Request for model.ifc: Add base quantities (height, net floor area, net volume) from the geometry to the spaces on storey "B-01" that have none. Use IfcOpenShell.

First a look at what the model holds.

```python
import ifcopenshell
import ifcopenshell.util.element
import ifcopenshell.util.unit

model = ifcopenshell.open("model.ifc")
print(model.schema)
for unit_type in ("LENGTHUNIT", "AREAUNIT", "VOLUMEUNIT"):
    print(unit_type, ifcopenshell.util.unit.calculate_unit_scale(model, unit_type))
storey = next(s for s in model.by_type("IfcBuildingStorey") if s.Name == "B-01")
spaces = [e for e in ifcopenshell.util.element.get_decomposition(storey) if e.is_a("IfcSpace")]
for e in sorted(spaces, key=lambda e: e.id()):
    print(e.id(), e.is_a(), e.Name, list(ifcopenshell.util.element.get_psets(e, qtos_only=True)), sep=" | ")
```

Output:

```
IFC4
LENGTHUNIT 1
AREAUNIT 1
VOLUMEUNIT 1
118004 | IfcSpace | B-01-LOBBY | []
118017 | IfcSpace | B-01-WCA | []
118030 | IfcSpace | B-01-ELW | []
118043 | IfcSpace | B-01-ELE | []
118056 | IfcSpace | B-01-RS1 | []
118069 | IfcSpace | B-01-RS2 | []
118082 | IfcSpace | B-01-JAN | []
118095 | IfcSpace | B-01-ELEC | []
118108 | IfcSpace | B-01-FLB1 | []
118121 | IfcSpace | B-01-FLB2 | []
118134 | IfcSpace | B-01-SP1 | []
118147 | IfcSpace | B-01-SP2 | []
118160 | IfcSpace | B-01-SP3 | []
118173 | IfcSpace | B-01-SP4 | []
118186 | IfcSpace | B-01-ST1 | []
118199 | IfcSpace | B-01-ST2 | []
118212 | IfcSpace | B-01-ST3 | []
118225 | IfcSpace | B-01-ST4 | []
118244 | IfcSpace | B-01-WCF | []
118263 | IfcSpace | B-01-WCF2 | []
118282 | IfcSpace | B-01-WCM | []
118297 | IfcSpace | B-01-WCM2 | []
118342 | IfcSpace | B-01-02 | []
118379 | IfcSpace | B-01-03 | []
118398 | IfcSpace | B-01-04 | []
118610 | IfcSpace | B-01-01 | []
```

```python
import ifcopenshell
import ifcopenshell.api.pset
import ifcopenshell.geom
import ifcopenshell.util.element
import ifcopenshell.util.shape
import ifcopenshell.util.unit

model = ifcopenshell.open("model.ifc")
unit_scale = ifcopenshell.util.unit.calculate_unit_scale(model)
area_scale = ifcopenshell.util.unit.calculate_unit_scale(model, "AREAUNIT")
volume_scale = ifcopenshell.util.unit.calculate_unit_scale(model, "VOLUMEUNIT")
settings = ifcopenshell.geom.settings()

storey = next(s for s in model.by_type("IfcBuildingStorey") if s.Name == "B-01")
spaces = [e for e in ifcopenshell.util.element.get_decomposition(storey) if e.is_a("IfcSpace")]

for e in sorted(spaces, key=lambda e: e.id()):
    if ifcopenshell.util.element.get_psets(e, qtos_only=True, should_inherit=False):
        continue
    # Geometry comes back in metres, in the element's own axes.
    shape = ifcopenshell.geom.create_shape(settings, e)
    values = {
        "Height": ifcopenshell.util.shape.get_z(shape.geometry) / unit_scale,
        "NetFloorArea": ifcopenshell.util.shape.get_footprint_area(shape.geometry) / area_scale,
        "NetVolume": ifcopenshell.util.shape.get_volume(shape.geometry) / volume_scale,
    }
    qto = ifcopenshell.api.pset.add_qto(model, product=e, name="Qto_SpaceBaseQuantities")
    ifcopenshell.api.pset.edit_qto(model, qto=qto, properties=values)
    print(e.id(), {k: round(v, 3) for k, v in values.items()})

model.write("model_rev.ifc")
```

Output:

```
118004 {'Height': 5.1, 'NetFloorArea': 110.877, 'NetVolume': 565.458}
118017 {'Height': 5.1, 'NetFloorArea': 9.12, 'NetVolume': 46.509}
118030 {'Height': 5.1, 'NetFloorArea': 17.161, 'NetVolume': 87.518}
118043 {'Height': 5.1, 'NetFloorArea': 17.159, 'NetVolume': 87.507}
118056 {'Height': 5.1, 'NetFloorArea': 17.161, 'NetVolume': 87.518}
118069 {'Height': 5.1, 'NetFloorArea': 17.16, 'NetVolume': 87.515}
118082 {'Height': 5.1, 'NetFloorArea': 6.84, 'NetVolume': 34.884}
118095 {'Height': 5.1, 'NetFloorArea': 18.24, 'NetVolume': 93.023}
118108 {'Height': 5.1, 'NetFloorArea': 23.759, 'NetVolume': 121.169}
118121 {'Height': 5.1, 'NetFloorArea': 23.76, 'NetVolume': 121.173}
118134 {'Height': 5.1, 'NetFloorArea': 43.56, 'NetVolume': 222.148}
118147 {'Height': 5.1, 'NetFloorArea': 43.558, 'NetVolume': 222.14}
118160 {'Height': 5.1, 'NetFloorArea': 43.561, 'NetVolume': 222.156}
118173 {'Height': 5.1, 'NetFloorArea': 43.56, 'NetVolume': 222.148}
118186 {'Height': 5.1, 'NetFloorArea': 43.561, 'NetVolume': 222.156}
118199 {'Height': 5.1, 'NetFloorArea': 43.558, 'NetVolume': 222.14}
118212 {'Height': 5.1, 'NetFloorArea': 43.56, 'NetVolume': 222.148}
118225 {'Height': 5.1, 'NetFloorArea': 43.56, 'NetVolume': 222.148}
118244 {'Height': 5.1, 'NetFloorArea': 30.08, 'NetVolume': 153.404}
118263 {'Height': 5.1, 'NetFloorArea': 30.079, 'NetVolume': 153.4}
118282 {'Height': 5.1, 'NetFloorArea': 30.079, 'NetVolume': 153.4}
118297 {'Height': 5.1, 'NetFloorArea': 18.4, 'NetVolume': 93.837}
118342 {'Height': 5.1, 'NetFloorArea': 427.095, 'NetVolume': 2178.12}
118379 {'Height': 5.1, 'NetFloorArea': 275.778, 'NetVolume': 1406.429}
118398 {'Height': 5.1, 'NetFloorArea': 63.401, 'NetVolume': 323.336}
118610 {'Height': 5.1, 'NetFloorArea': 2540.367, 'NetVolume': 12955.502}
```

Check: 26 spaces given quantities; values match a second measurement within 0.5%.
